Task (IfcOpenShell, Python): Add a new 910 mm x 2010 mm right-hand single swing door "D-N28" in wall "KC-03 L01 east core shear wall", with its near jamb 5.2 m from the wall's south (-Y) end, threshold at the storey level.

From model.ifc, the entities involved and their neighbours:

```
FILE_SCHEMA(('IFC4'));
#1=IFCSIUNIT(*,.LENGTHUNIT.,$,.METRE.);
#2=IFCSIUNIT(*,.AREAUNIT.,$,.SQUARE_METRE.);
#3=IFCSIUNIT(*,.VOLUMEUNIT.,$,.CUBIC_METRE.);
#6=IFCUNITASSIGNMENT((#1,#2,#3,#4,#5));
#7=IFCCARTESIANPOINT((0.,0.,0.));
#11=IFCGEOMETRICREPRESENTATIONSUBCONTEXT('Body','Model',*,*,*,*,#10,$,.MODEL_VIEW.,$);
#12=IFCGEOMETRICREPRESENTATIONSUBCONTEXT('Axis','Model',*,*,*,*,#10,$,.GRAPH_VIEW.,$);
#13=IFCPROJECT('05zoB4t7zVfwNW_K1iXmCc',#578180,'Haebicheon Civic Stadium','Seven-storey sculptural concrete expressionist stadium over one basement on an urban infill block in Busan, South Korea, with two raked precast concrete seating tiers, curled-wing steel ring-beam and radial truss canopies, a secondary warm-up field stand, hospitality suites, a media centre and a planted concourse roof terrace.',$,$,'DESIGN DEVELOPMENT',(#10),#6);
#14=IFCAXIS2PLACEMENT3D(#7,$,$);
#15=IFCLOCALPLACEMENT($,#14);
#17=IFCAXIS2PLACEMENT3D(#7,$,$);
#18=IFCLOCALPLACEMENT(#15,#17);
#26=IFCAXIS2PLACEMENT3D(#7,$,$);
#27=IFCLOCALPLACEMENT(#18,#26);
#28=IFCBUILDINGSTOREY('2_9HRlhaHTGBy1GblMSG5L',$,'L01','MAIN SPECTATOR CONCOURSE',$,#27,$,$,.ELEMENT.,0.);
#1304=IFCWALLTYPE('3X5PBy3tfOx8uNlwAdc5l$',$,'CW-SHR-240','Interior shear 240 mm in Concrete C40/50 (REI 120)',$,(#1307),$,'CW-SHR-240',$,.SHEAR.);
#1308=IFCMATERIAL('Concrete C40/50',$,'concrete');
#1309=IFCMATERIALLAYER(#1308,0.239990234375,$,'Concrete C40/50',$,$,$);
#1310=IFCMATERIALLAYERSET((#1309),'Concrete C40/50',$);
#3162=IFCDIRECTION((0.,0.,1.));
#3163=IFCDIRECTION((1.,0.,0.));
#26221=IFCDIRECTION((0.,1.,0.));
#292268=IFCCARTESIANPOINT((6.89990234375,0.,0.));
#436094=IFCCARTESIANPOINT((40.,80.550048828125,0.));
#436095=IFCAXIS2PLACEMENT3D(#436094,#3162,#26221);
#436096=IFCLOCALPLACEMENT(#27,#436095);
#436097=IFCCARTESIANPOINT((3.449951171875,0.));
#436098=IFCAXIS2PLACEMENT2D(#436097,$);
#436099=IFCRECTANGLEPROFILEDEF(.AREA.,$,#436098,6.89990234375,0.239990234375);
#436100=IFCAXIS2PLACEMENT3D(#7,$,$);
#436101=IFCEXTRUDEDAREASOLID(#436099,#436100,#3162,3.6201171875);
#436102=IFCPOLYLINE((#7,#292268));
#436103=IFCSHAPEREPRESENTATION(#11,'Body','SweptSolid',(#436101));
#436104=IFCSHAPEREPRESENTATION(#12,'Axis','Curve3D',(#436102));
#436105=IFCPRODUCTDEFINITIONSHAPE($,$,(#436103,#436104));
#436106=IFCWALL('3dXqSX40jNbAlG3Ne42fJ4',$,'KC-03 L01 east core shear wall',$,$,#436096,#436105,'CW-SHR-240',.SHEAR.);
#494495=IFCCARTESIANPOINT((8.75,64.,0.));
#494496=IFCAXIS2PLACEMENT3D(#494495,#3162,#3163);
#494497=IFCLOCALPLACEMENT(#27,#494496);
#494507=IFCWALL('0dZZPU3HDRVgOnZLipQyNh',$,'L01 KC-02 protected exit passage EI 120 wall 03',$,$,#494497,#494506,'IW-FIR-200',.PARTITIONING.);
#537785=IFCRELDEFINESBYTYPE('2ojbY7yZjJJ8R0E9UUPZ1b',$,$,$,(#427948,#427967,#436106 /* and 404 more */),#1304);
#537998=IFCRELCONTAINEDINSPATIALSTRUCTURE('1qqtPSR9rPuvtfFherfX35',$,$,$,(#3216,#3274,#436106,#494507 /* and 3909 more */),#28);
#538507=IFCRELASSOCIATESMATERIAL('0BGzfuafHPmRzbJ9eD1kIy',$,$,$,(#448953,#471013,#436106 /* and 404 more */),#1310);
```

```python
import numpy as np
import ifcopenshell
import ifcopenshell.api.feature
import ifcopenshell.api.geometry
import ifcopenshell.api.root
import ifcopenshell.api.spatial
import ifcopenshell.geom
import ifcopenshell.util.element
import ifcopenshell.util.placement
import ifcopenshell.util.representation
import ifcopenshell.util.shape
import ifcopenshell.util.unit

model = ifcopenshell.open("model.ifc")
unit_scale = ifcopenshell.util.unit.calculate_unit_scale(model)
settings = ifcopenshell.geom.settings()


def volume(element):
    """Net volume in cubic metres, openings subtracted."""
    shape = ifcopenshell.geom.create_shape(settings, element)
    return ifcopenshell.util.shape.get_volume(shape.geometry)


wall = model.by_guid("3dXqSX40jNbAlG3Ne42fJ4")
storey = ifcopenshell.util.element.get_container(wall, ifc_class="IfcBuildingStorey")
context = ifcopenshell.util.representation.get_context(model, "Model", "Body", "MODEL_VIEW")
before = volume(wall)

width, height, from_end, sill = 0.91, 2.01, 5.2, 0.0  # metres

# The wall runs along its own X axis, and the end named is its -X end.
wall_shape = ifcopenshell.geom.create_shape(settings, wall)
x, y, z = ifcopenshell.util.shape.get_vertices(wall_shape.geometry).T
start = x.min() + from_end
face, thickness = float(y.min()), float(y.max() - y.min())
wall_matrix = ifcopenshell.util.placement.get_local_placement(wall.ObjectPlacement)
level = ifcopenshell.util.placement.get_local_placement(storey.ObjectPlacement)[2, 3]


def in_wall(x, y):
    """Placement at x, y metres in the wall's axes, at sill height."""
    matrix = wall_matrix.copy()
    matrix[:, 3] = wall_matrix @ np.array([x / unit_scale, y / unit_scale, 0.0, 1.0])
    matrix[2, 3] = level + sill / unit_scale
    return matrix


# Opening: a box that overshoots both wall faces by 50 mm.
opening = ifcopenshell.api.root.create_entity(model, ifc_class="IfcOpeningElement", predefined_type="OPENING")
box = ifcopenshell.api.geometry.add_wall_representation(
    model, context=context, length=width, height=height, thickness=thickness + 0.1
)
ifcopenshell.api.geometry.assign_representation(model, product=opening, representation=box)
ifcopenshell.api.geometry.edit_object_placement(model, product=opening, matrix=in_wall(start, face - 0.05), is_si=False)
ifcopenshell.api.feature.add_feature(model, feature=opening, element=wall)

door = ifcopenshell.api.root.create_entity(model, ifc_class="IfcDoor", name="D-N28", predefined_type="DOOR")
door.OverallWidth, door.OverallHeight = width / unit_scale, height / unit_scale
door.OperationType = "SINGLE_SWING_RIGHT"
body = ifcopenshell.api.geometry.add_door_representation(
    model,
    context=context,
    overall_width=door.OverallWidth,
    overall_height=door.OverallHeight,
    operation_type="SINGLE_SWING_RIGHT",
    lining_properties={"LiningDepth": thickness / unit_scale, "ThresholdDepth": thickness / unit_scale},
)
ifcopenshell.api.geometry.assign_representation(model, product=door, representation=body)
ifcopenshell.api.spatial.assign_container(model, products=[door], relating_structure=storey)
ifcopenshell.api.feature.add_filling(model, opening=opening, element=door)

# The lining spans the wall, so the door starts at the wall face.
ifcopenshell.api.geometry.edit_object_placement(model, product=door, matrix=in_wall(start, face), is_si=False)

after = volume(wall)

print(f"wall volume {before:.3f} -> {after:.3f} m3")

model.write("model_rev.ifc")
```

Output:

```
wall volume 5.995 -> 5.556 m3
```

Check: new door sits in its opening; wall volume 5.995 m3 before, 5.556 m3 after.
